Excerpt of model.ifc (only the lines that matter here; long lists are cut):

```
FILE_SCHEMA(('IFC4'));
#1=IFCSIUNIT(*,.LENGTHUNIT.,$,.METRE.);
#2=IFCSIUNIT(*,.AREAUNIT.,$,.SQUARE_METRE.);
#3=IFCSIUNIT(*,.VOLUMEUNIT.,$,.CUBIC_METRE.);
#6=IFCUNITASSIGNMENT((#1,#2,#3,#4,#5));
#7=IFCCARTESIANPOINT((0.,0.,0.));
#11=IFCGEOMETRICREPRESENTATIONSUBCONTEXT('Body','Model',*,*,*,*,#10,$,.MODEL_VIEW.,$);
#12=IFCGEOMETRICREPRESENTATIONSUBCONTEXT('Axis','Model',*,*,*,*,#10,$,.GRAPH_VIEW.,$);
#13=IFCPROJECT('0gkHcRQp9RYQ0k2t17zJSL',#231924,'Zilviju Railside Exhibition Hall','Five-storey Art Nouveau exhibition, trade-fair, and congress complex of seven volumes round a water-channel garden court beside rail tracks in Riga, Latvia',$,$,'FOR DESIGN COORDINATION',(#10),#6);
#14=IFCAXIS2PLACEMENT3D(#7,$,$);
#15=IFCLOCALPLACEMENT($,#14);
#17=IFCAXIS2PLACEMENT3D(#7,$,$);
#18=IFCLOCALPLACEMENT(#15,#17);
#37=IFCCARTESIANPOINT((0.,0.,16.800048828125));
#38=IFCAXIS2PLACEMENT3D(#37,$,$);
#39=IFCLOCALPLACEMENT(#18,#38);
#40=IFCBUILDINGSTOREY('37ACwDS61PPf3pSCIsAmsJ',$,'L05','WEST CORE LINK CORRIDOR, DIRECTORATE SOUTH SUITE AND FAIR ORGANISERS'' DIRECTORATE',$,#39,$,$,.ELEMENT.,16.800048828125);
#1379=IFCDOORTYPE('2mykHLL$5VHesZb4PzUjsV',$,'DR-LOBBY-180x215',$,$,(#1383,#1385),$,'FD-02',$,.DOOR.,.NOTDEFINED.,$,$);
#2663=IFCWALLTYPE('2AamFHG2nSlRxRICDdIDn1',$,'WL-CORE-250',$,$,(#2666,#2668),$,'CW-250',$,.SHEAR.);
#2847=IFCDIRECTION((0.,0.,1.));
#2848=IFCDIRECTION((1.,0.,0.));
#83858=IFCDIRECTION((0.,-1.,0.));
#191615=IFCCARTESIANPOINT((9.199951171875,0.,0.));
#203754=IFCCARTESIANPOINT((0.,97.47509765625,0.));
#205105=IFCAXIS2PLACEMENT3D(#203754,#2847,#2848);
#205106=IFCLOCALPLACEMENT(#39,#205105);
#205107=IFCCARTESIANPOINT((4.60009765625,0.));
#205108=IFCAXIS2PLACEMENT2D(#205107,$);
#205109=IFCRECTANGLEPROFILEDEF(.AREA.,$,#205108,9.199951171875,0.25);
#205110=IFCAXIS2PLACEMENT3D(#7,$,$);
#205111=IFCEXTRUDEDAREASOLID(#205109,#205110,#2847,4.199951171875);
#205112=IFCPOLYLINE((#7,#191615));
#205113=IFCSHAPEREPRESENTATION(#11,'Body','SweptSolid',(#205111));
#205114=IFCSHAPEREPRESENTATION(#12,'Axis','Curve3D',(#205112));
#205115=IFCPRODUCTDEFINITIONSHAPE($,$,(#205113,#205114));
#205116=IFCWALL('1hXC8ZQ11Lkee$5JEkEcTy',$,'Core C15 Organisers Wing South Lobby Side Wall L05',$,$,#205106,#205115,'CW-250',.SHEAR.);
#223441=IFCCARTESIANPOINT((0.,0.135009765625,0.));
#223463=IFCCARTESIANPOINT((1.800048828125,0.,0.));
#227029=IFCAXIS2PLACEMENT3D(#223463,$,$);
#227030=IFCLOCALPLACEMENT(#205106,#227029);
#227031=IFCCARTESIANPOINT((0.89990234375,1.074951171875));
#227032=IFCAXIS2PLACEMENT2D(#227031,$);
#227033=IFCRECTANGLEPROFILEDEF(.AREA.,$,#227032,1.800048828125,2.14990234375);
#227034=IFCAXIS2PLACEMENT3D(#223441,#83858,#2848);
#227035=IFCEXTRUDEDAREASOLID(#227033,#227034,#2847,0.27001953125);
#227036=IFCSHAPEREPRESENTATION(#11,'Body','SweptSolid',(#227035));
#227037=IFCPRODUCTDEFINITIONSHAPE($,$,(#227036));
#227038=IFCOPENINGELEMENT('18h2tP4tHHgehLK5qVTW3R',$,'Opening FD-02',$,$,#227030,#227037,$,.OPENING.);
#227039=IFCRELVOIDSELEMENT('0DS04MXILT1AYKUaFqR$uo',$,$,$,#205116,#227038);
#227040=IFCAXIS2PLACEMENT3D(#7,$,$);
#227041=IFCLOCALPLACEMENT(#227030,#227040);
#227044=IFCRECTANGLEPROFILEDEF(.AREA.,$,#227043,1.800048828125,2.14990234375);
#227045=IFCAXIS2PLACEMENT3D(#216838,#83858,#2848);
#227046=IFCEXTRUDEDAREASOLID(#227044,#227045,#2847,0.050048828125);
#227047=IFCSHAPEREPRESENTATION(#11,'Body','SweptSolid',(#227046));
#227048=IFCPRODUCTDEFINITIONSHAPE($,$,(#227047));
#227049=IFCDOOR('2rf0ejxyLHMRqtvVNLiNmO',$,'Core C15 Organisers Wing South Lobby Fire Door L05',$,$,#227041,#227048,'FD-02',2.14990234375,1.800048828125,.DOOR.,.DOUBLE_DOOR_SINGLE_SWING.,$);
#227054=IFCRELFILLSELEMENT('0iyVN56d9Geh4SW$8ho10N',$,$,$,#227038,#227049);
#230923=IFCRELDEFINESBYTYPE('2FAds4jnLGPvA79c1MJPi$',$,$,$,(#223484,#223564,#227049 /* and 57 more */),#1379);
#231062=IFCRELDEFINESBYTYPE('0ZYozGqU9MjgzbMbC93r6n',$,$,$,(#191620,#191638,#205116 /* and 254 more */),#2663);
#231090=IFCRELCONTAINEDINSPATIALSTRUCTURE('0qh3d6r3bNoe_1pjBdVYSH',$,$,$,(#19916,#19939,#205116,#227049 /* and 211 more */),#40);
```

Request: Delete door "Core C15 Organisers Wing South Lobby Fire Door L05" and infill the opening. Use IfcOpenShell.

```python
import ifcopenshell
import ifcopenshell.api.feature
import ifcopenshell.api.root
import ifcopenshell.geom
import ifcopenshell.util.shape

model = ifcopenshell.open("model.ifc")
settings = ifcopenshell.geom.settings()


def volume(element):
    """Net volume in cubic metres, openings subtracted."""
    shape = ifcopenshell.geom.create_shape(settings, element)
    return ifcopenshell.util.shape.get_volume(shape.geometry)


door = model.by_guid("2rf0ejxyLHMRqtvVNLiNmO")
opening = door.FillsVoids[0].RelatingOpeningElement
wall = opening.VoidsElements[0].RelatingBuildingElement
before = volume(wall)

ifcopenshell.api.root.remove_product(model, product=door)
ifcopenshell.api.feature.remove_feature(model, feature=opening)

after = volume(wall)

print(f"wall volume {before:.3f} -> {after:.3f} m3")

model.write("model-out.ifc")
```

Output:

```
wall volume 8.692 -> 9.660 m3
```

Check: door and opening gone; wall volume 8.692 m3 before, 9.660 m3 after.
